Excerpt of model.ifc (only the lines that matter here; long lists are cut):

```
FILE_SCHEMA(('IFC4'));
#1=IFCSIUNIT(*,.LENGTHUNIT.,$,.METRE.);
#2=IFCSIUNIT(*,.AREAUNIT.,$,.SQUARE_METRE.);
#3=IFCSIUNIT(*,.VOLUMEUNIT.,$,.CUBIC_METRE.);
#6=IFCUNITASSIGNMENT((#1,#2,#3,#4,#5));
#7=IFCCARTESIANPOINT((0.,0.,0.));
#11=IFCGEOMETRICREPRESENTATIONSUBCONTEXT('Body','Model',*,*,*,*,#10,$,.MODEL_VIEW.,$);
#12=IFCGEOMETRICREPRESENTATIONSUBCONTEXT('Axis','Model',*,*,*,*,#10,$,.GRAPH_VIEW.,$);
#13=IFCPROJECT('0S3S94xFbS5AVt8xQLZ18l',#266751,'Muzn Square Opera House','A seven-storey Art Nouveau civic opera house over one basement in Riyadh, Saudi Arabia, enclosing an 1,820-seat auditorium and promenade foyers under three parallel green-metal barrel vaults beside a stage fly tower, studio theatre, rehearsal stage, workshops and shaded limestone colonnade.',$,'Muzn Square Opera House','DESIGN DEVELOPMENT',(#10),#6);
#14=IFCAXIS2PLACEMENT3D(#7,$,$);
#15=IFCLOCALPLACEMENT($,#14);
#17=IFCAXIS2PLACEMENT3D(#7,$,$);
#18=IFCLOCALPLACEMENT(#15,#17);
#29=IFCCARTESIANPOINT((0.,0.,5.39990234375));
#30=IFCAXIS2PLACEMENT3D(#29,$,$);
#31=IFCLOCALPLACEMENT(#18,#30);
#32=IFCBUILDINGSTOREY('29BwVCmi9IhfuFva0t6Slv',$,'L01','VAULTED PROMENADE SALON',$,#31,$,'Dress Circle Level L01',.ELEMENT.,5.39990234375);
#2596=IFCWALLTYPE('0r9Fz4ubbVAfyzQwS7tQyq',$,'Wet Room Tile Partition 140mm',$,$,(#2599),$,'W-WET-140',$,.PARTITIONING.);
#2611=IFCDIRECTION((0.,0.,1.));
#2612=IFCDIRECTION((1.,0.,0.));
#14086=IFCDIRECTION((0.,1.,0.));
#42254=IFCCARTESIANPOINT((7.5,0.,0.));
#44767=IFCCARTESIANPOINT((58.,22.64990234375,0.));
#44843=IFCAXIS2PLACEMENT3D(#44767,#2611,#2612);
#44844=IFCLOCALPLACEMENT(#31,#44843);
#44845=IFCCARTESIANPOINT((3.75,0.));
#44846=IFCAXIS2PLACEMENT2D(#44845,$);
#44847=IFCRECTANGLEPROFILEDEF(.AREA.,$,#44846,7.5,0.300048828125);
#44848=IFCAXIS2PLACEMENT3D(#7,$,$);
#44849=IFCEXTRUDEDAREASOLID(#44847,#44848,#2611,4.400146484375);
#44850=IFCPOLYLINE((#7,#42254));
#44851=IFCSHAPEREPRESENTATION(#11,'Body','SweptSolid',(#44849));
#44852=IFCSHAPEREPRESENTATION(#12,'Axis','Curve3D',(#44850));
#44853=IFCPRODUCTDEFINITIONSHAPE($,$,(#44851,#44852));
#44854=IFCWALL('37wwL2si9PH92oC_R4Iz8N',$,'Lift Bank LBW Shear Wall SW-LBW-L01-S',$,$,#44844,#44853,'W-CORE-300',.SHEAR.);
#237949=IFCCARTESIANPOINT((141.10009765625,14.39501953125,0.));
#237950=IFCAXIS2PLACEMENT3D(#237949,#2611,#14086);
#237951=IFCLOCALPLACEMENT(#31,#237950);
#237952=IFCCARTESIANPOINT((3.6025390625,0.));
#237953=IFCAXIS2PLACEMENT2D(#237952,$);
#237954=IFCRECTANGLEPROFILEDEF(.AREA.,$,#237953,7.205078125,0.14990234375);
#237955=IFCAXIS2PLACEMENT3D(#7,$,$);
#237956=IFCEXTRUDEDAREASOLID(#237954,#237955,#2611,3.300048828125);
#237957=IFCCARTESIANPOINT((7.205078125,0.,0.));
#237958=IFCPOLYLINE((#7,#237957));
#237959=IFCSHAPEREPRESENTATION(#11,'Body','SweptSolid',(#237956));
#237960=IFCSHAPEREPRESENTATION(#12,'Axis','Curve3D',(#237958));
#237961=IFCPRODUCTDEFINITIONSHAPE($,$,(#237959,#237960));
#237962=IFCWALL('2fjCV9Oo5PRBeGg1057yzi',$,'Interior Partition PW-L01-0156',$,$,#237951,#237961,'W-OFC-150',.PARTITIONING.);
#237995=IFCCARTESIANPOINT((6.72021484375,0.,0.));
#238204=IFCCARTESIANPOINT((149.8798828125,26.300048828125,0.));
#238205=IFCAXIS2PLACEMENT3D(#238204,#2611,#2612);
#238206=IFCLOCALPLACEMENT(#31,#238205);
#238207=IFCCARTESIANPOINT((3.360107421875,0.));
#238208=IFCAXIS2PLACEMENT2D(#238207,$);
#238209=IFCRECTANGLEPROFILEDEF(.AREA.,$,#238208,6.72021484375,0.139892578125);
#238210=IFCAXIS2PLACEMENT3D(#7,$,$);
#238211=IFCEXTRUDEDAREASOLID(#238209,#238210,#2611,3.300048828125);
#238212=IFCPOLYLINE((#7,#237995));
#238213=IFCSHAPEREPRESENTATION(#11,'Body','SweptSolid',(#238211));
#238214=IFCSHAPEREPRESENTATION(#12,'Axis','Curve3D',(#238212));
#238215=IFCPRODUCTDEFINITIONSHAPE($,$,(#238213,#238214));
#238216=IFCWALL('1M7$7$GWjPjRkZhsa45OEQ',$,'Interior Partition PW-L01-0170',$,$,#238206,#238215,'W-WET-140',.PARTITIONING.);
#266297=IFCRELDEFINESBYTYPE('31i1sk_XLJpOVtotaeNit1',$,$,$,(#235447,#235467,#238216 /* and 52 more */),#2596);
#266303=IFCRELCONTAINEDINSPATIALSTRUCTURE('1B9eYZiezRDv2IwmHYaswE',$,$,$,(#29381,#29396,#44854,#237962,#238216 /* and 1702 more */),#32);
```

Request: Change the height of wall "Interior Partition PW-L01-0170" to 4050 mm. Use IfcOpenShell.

```python
import ifcopenshell
import ifcopenshell.geom
import ifcopenshell.util.representation
import ifcopenshell.util.shape
import ifcopenshell.util.unit

model = ifcopenshell.open("model.ifc")
unit_scale = ifcopenshell.util.unit.calculate_unit_scale(model)
settings = ifcopenshell.geom.settings()


def volume(element):
    """Net volume in cubic metres, openings subtracted."""
    shape = ifcopenshell.geom.create_shape(settings, element)
    return ifcopenshell.util.shape.get_volume(shape.geometry)


wall = model.by_guid("1M7$7$GWjPjRkZhsa45OEQ")
before = volume(wall)

body = ifcopenshell.util.representation.get_representation(wall, "Model", "Body")
solid = body.Items[0]
old_height = solid.Depth
solid.Depth = 4.05 / unit_scale
after = volume(wall)

print(f"height {old_height:g} -> {solid.Depth:g}, volume {before:.3f} -> {after:.3f} m3")

model.write("model-out.ifc")
```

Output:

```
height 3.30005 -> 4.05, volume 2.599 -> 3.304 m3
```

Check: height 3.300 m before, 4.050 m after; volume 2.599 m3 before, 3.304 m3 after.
